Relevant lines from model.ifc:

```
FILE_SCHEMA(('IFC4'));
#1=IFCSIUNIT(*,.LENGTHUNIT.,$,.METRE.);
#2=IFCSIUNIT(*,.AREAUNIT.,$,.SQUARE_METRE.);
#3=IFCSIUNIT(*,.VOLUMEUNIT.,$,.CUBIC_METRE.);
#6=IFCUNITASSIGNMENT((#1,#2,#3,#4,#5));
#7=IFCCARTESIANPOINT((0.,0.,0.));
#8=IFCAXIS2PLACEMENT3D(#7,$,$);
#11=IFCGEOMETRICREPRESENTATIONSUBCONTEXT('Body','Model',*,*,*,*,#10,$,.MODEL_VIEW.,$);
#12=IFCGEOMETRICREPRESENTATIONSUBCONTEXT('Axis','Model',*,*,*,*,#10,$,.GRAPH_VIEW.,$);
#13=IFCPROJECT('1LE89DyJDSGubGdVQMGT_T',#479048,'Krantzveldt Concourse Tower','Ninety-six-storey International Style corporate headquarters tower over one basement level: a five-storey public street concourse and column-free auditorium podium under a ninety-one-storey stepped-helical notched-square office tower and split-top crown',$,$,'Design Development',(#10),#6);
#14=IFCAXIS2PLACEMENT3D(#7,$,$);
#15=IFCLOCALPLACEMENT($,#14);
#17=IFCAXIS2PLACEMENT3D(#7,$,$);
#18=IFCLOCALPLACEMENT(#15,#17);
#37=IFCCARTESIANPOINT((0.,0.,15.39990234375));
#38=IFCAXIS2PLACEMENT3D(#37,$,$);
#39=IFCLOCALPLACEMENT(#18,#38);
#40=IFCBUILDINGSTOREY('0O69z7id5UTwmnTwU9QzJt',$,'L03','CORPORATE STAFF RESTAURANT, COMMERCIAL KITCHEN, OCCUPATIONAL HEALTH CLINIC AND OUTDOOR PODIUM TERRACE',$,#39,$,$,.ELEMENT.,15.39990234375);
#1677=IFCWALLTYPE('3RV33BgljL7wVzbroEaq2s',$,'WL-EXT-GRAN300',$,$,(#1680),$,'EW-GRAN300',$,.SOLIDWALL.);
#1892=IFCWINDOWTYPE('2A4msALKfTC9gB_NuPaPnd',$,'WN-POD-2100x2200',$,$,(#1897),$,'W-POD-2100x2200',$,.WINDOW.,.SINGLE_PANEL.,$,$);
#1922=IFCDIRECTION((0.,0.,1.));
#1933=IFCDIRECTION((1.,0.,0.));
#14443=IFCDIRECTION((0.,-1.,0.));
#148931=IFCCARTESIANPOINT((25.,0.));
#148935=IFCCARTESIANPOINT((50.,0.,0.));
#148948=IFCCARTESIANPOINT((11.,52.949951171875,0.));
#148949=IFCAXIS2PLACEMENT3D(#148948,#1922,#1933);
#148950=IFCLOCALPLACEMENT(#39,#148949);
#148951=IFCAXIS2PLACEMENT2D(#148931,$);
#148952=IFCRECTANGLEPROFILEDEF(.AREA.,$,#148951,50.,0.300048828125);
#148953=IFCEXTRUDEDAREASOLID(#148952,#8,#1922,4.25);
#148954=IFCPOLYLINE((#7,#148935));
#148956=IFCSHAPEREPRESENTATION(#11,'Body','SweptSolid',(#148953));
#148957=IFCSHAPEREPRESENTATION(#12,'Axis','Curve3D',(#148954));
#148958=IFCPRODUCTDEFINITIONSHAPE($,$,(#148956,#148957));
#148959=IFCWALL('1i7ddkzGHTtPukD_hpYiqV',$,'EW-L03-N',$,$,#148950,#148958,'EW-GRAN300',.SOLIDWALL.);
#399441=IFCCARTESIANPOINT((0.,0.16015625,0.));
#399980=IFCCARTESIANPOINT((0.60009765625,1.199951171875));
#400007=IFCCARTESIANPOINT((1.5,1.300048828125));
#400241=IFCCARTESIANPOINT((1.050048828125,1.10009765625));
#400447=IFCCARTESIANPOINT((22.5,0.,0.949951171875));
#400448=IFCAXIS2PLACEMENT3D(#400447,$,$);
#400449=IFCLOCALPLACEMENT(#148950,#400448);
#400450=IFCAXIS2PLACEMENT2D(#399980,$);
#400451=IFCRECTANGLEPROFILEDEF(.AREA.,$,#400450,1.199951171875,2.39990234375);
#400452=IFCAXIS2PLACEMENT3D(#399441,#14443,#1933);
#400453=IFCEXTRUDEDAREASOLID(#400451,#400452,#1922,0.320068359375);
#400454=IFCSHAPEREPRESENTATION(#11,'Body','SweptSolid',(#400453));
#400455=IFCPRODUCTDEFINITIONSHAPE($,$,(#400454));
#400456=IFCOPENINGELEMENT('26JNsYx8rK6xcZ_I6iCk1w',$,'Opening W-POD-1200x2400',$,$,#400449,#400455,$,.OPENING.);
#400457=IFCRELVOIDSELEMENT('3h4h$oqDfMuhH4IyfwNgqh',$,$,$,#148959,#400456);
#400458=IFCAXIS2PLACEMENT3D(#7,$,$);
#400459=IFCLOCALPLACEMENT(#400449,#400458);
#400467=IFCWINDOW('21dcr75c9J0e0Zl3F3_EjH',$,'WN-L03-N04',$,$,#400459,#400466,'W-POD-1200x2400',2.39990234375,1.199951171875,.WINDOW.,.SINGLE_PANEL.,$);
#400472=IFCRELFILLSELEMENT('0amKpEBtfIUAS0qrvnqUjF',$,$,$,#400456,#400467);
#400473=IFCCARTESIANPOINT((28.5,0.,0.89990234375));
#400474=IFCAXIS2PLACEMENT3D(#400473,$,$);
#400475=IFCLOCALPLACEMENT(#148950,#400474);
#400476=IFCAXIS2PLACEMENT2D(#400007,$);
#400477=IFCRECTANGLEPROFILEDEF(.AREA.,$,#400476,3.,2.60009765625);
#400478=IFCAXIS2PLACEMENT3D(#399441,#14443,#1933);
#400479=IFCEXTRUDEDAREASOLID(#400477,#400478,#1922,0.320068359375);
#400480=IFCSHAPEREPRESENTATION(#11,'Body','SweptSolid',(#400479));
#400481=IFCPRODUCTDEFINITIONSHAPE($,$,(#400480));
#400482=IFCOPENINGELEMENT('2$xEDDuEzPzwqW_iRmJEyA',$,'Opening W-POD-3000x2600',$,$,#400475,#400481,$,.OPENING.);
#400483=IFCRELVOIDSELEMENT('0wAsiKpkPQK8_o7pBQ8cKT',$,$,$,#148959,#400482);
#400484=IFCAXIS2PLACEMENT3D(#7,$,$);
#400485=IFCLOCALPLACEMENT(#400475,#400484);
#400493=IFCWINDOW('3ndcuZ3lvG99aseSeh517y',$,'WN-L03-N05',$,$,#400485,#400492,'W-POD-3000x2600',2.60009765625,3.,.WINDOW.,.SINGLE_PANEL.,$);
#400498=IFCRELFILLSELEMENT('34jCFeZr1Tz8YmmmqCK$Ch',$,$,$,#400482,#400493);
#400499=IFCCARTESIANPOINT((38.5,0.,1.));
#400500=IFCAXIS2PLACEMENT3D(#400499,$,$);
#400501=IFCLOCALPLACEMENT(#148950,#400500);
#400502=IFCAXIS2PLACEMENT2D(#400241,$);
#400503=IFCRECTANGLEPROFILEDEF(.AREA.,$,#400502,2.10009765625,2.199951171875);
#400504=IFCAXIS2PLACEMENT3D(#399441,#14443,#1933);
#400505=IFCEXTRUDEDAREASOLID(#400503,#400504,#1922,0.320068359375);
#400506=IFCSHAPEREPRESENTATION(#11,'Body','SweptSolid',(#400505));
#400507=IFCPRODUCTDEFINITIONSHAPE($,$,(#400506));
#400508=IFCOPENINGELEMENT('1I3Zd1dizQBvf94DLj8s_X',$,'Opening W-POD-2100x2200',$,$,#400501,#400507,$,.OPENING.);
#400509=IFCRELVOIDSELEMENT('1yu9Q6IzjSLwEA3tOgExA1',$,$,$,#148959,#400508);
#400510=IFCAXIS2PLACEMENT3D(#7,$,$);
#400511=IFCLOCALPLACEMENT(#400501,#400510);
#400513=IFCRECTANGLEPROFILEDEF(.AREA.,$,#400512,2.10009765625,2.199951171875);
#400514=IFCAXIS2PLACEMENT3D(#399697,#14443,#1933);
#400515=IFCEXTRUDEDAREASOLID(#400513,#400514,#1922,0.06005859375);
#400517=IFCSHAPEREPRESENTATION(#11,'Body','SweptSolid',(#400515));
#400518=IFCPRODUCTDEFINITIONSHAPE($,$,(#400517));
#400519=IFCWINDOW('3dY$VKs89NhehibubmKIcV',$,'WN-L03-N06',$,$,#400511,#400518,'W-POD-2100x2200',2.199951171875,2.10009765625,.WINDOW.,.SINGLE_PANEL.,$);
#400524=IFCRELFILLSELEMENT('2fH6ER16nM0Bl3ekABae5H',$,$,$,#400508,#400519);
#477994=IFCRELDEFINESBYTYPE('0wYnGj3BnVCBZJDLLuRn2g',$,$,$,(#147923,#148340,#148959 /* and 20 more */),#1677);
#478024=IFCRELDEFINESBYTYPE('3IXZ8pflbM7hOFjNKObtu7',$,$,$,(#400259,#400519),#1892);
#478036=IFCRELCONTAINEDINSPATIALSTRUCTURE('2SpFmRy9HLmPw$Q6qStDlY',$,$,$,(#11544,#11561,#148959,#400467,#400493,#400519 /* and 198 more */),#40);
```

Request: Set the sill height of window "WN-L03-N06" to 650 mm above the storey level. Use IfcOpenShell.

```python
import numpy as np
import ifcopenshell
import ifcopenshell.api.geometry
import ifcopenshell.geom
import ifcopenshell.util.element
import ifcopenshell.util.placement
import ifcopenshell.util.shape
import ifcopenshell.util.unit

model = ifcopenshell.open("model.ifc")
unit_scale = ifcopenshell.util.unit.calculate_unit_scale(model)

window = model.by_id(400519)
opening = window.FillsVoids[0].RelatingOpeningElement
storey = ifcopenshell.util.element.get_container(window, ifc_class="IfcBuildingStorey")
level = ifcopenshell.util.placement.get_local_placement(storey.ObjectPlacement)[2, 3]

# The opening's origin need not be at the sill, so measure its lowest point.
shape = ifcopenshell.geom.create_shape(ifcopenshell.geom.settings(), opening)
bottom = ifcopenshell.util.shape.get_shape_bottom_elevation(shape, shape.geometry) / unit_scale
dz = level + 0.65 - bottom

shift = np.array([0.0, 0.0, dz])
# The window is placed relative to its opening, so it follows when the opening moves.
matrix = ifcopenshell.util.placement.get_local_placement(opening.ObjectPlacement)
matrix[:3, 3] += shift
ifcopenshell.api.geometry.edit_object_placement(
    model, product=opening, matrix=matrix, is_si=False, should_transform_children=True
)

print(f"moved by {dz * unit_scale:+.3f} m")

model.write("model-out.ifc")
```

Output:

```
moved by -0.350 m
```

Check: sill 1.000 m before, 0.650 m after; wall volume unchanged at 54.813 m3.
